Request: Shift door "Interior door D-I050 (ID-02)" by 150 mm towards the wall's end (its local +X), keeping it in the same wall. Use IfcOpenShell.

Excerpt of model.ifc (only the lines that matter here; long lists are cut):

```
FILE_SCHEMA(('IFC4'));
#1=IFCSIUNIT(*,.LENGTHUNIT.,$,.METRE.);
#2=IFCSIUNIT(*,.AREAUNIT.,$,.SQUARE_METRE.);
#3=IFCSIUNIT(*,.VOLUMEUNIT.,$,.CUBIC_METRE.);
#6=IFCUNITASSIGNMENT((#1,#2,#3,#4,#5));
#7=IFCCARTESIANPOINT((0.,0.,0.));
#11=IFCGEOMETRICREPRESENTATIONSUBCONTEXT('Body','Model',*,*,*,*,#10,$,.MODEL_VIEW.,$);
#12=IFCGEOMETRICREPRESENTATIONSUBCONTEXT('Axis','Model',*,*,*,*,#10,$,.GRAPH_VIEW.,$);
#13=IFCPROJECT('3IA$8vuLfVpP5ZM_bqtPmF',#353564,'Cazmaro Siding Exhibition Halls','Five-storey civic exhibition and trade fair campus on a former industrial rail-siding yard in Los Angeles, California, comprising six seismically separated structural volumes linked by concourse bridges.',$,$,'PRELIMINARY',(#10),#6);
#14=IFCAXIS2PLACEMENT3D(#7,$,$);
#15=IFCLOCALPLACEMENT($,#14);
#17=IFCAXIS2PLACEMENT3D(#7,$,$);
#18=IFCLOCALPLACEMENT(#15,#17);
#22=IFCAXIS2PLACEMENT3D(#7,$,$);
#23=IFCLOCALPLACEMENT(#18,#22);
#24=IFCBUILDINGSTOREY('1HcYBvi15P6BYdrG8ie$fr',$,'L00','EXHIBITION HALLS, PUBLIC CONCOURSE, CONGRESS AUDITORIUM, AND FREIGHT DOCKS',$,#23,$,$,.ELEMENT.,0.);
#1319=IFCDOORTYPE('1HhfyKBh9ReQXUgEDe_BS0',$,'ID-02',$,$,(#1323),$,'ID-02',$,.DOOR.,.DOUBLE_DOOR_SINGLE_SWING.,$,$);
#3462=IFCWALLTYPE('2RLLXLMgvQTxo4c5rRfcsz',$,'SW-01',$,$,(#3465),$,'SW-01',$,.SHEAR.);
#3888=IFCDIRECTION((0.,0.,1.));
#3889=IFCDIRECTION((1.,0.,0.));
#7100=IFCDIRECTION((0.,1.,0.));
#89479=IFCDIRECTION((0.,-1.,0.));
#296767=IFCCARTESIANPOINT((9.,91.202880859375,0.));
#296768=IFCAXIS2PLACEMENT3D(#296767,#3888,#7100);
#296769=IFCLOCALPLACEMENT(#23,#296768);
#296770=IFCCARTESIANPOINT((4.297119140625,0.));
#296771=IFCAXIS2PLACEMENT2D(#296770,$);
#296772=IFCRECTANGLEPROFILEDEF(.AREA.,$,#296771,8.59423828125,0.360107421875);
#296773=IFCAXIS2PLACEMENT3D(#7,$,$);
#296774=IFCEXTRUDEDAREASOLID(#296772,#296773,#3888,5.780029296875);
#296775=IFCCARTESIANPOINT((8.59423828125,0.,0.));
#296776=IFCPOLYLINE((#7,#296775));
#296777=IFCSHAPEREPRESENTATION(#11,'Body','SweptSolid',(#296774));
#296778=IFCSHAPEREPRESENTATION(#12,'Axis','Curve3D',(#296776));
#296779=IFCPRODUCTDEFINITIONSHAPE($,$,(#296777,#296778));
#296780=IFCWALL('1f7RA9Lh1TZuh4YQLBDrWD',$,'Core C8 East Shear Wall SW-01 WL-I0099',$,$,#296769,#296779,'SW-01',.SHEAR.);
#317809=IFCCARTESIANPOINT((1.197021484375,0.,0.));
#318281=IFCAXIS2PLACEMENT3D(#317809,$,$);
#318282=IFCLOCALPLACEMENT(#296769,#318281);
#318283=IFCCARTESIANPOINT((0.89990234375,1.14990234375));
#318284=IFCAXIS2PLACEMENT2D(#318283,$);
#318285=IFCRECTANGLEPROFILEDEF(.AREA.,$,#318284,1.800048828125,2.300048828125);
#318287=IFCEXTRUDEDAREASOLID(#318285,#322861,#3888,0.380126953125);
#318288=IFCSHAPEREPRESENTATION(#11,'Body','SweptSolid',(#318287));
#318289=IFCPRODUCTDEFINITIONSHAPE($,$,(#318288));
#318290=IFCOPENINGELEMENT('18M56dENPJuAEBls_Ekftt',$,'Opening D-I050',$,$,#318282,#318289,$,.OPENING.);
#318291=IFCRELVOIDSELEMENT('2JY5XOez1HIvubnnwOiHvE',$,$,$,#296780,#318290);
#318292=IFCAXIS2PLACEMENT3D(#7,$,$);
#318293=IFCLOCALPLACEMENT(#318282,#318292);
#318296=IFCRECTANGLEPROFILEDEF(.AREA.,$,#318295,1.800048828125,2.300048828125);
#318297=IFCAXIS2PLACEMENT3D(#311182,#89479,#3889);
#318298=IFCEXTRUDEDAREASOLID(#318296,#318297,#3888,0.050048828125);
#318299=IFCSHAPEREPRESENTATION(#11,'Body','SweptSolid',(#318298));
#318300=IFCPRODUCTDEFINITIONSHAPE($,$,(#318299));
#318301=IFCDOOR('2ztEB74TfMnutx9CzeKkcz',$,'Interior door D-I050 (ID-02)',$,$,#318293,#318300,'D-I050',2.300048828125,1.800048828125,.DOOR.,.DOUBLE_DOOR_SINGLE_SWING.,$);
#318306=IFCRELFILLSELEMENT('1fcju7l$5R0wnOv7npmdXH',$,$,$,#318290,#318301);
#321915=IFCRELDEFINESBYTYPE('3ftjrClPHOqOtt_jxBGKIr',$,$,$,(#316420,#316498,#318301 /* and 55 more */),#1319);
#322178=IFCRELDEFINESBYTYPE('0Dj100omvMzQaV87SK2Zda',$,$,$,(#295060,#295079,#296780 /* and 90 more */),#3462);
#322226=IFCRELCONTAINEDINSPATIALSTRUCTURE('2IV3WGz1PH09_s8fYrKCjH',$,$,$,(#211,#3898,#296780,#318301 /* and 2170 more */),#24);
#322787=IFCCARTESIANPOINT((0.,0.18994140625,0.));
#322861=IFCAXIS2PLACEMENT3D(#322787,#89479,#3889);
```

```python
import ifcopenshell
import ifcopenshell.api.geometry
import ifcopenshell.util.placement
import ifcopenshell.util.unit

model = ifcopenshell.open("model.ifc")
unit_scale = ifcopenshell.util.unit.calculate_unit_scale(model)

door = model.by_guid("2ztEB74TfMnutx9CzeKkcz")
opening = door.FillsVoids[0].RelatingOpeningElement
wall = opening.VoidsElements[0].RelatingBuildingElement

wall_matrix = ifcopenshell.util.placement.get_local_placement(wall.ObjectPlacement)
shift = wall_matrix[:3, 0] * 0.15 / unit_scale
before = ifcopenshell.util.placement.get_local_placement(door.ObjectPlacement)[:3, 3].copy()

# The door is placed relative to its opening, so it follows when the opening moves.
matrix = ifcopenshell.util.placement.get_local_placement(opening.ObjectPlacement)
matrix[:3, 3] += shift
ifcopenshell.api.geometry.edit_object_placement(
    model, product=opening, matrix=matrix, is_si=False, should_transform_children=True
)

after = ifcopenshell.util.placement.get_local_placement(door.ObjectPlacement)[:3, 3]
print("door moved by", (after - before).round(3) + 0.0)

model.write("model_updated.ifc")
```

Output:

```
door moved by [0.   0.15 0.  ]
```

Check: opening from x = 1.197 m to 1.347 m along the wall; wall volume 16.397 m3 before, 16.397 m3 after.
